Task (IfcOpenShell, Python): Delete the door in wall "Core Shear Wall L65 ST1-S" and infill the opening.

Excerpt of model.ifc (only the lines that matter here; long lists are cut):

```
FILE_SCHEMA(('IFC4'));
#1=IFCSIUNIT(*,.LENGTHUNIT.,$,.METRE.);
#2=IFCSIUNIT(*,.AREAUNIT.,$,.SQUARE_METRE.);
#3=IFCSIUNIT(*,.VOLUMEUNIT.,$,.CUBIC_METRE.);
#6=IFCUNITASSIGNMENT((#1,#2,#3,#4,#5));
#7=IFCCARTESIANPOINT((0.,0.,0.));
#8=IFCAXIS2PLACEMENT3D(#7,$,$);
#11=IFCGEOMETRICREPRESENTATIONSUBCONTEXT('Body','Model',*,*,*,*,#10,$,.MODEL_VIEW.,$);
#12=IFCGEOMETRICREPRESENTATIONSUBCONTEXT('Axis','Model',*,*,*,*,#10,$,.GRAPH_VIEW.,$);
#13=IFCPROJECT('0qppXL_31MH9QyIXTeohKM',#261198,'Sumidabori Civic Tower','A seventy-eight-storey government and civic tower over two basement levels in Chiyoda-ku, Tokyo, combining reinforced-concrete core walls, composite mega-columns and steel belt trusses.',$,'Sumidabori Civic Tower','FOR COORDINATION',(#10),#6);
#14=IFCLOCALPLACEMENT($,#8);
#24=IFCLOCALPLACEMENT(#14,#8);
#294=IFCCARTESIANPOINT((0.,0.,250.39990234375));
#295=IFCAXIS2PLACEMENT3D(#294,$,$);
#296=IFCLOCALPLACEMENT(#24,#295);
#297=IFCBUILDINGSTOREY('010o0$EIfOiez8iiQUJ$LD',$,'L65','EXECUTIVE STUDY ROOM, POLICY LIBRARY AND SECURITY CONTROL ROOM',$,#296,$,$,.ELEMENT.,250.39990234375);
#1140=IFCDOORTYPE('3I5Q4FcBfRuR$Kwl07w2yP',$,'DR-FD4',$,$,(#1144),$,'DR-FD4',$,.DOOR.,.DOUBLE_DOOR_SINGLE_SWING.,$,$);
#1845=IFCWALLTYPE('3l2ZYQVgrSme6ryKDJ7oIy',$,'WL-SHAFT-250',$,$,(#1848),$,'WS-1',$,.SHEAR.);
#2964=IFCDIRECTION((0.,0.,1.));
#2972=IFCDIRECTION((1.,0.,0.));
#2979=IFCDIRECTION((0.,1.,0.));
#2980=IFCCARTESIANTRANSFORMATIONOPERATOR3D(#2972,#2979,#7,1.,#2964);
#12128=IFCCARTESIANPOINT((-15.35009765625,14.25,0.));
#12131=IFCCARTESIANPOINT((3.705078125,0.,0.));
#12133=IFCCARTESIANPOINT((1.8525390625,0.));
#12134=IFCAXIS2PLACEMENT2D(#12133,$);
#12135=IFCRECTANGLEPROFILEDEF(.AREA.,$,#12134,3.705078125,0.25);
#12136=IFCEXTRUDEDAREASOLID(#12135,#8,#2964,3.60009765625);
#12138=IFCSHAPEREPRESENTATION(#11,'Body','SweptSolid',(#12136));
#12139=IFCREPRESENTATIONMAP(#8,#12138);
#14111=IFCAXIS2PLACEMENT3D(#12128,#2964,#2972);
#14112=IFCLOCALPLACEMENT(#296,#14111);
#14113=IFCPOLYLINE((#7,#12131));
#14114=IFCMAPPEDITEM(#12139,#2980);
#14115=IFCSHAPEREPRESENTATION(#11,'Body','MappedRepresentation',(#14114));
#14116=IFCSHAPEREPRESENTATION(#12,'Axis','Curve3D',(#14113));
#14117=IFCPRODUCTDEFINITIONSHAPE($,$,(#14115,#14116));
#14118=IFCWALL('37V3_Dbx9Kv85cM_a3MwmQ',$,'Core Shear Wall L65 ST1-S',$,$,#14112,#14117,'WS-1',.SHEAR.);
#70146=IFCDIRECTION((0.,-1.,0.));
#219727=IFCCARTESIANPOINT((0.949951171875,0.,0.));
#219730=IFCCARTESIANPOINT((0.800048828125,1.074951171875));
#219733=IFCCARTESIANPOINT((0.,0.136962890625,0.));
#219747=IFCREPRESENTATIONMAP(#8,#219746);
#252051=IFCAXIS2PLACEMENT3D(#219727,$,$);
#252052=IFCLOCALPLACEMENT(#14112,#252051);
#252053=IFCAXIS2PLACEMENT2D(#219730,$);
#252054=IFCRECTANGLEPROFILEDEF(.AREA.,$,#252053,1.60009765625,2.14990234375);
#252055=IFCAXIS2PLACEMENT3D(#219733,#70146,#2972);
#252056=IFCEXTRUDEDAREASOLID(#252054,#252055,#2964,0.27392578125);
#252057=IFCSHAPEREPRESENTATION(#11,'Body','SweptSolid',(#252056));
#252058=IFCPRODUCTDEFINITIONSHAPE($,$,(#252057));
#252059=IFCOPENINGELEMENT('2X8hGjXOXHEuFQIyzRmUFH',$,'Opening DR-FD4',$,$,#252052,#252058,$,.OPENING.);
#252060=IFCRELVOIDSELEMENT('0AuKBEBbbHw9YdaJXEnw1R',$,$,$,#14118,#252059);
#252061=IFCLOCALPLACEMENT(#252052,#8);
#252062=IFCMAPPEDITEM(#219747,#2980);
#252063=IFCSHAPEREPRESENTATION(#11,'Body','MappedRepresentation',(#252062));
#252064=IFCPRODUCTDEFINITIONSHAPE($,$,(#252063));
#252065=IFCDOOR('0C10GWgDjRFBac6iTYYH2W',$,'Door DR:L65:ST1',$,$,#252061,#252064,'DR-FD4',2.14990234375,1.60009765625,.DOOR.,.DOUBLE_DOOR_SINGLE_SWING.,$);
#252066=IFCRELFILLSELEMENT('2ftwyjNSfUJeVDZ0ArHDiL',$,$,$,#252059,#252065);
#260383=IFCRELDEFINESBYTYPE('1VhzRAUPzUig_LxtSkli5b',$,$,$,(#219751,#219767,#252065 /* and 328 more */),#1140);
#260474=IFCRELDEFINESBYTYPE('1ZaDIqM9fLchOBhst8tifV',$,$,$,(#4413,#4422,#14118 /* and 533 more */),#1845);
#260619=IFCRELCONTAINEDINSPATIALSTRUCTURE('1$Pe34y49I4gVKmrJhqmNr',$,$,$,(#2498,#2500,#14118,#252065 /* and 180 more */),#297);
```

```python
import ifcopenshell
import ifcopenshell.api.feature
import ifcopenshell.api.root
import ifcopenshell.geom
import ifcopenshell.util.shape

model = ifcopenshell.open("model.ifc")
settings = ifcopenshell.geom.settings()


def volume(element):
    """Net volume in cubic metres, openings subtracted."""
    shape = ifcopenshell.geom.create_shape(settings, element)
    return ifcopenshell.util.shape.get_volume(shape.geometry)


door = model.by_guid("0C10GWgDjRFBac6iTYYH2W")
opening = door.FillsVoids[0].RelatingOpeningElement
wall = opening.VoidsElements[0].RelatingBuildingElement
before = volume(wall)

ifcopenshell.api.root.remove_product(model, product=door)
ifcopenshell.api.feature.remove_feature(model, feature=opening)

after = volume(wall)

print(f"wall volume {before:.3f} -> {after:.3f} m3")

model.write("model_v2.ifc")
```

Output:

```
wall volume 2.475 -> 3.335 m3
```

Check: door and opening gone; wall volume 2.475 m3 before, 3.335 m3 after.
